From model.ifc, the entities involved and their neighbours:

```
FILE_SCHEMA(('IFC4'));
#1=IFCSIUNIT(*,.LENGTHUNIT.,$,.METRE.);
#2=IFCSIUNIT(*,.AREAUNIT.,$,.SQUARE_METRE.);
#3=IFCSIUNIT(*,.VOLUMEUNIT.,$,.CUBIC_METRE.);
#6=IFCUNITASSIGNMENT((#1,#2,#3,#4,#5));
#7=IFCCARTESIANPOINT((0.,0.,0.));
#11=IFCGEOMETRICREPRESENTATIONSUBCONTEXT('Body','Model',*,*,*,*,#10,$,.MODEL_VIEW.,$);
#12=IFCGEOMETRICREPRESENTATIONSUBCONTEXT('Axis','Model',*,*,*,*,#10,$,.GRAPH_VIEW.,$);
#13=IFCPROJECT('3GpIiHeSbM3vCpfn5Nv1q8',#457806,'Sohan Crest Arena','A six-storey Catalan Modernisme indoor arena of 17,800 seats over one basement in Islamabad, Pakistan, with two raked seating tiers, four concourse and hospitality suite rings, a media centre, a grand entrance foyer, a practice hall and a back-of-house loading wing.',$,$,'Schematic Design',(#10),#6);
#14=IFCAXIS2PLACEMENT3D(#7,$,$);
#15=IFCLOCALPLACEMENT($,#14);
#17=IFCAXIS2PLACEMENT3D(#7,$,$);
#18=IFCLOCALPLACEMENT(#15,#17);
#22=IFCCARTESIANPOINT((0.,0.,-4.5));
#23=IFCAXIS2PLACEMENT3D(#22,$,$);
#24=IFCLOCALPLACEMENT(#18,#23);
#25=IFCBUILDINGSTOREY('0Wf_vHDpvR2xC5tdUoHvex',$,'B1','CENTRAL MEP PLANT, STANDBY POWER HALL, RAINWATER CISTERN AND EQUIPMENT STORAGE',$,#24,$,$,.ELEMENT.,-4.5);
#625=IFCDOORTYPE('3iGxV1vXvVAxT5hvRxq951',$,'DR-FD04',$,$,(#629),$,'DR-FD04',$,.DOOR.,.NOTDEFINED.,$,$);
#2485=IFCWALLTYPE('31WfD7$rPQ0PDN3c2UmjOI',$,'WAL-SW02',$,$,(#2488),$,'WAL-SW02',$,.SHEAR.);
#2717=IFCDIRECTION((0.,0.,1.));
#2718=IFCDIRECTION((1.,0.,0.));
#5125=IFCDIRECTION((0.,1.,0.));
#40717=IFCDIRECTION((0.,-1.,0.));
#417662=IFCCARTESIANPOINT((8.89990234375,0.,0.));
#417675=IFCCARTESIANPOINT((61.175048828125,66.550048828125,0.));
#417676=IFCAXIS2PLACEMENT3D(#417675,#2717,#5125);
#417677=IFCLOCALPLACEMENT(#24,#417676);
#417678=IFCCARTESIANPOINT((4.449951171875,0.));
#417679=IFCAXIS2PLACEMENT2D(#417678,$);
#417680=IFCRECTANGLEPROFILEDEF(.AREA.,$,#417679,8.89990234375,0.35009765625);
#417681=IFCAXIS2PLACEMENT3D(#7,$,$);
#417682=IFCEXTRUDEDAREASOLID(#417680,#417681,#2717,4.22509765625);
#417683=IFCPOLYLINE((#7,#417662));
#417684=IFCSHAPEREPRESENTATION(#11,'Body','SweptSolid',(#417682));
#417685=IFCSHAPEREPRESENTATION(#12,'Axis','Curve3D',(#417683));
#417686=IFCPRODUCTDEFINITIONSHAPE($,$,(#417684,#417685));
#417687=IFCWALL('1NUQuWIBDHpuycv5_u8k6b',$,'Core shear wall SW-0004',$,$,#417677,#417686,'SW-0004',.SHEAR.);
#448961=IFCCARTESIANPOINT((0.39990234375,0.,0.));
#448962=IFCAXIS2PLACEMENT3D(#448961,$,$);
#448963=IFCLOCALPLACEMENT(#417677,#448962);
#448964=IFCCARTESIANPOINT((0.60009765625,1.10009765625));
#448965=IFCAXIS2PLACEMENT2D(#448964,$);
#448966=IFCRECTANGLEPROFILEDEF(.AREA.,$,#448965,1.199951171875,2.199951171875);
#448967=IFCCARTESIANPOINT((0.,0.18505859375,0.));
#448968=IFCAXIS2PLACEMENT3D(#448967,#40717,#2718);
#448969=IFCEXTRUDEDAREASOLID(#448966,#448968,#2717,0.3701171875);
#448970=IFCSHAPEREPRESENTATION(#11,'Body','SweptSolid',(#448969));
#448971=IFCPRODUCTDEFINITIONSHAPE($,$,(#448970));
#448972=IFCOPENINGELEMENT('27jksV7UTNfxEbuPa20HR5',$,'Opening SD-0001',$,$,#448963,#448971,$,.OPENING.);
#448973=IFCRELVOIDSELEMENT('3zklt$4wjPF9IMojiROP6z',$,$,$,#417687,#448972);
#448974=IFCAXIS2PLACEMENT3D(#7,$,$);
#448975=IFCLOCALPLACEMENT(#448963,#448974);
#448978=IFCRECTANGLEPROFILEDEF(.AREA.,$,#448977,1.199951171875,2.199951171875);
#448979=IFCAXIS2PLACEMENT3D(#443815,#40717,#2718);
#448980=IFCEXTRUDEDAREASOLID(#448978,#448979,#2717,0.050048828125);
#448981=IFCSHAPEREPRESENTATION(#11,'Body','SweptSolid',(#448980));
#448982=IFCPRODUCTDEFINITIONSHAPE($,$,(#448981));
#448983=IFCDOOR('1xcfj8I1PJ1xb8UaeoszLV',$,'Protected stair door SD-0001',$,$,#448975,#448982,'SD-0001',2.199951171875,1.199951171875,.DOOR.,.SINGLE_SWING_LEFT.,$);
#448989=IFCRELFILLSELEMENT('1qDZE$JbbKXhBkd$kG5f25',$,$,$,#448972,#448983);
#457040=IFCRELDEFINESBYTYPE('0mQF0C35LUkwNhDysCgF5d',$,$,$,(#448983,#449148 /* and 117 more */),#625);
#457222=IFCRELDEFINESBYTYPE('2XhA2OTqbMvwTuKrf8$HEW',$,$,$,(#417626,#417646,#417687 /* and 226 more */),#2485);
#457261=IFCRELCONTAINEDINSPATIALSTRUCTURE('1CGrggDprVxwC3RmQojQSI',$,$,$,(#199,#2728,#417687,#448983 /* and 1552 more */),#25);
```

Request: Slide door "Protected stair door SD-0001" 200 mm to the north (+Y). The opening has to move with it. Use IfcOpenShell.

```python
import ifcopenshell
import ifcopenshell.api.geometry
import ifcopenshell.util.placement

model = ifcopenshell.open("model.ifc")

door = model.by_id(448983)
opening = door.FillsVoids[0].RelatingOpeningElement
wall = opening.VoidsElements[0].RelatingBuildingElement

wall_matrix = ifcopenshell.util.placement.get_local_placement(wall.ObjectPlacement)
shift = wall_matrix[:3, 0] * 0.2
before = ifcopenshell.util.placement.get_local_placement(door.ObjectPlacement)[:3, 3].copy()

# The door is placed relative to its opening, so it follows when the opening moves.
matrix = ifcopenshell.util.placement.get_local_placement(opening.ObjectPlacement)
matrix[:3, 3] += shift
ifcopenshell.api.geometry.edit_object_placement(
    model, product=opening, matrix=matrix, is_si=False, should_transform_children=True
)

after = ifcopenshell.util.placement.get_local_placement(door.ObjectPlacement)[:3, 3]
print("door moved by", (after - before).round(3) + 0.0)

model.write("model-out.ifc")
```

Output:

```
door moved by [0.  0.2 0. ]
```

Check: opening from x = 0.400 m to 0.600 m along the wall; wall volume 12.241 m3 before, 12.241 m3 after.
